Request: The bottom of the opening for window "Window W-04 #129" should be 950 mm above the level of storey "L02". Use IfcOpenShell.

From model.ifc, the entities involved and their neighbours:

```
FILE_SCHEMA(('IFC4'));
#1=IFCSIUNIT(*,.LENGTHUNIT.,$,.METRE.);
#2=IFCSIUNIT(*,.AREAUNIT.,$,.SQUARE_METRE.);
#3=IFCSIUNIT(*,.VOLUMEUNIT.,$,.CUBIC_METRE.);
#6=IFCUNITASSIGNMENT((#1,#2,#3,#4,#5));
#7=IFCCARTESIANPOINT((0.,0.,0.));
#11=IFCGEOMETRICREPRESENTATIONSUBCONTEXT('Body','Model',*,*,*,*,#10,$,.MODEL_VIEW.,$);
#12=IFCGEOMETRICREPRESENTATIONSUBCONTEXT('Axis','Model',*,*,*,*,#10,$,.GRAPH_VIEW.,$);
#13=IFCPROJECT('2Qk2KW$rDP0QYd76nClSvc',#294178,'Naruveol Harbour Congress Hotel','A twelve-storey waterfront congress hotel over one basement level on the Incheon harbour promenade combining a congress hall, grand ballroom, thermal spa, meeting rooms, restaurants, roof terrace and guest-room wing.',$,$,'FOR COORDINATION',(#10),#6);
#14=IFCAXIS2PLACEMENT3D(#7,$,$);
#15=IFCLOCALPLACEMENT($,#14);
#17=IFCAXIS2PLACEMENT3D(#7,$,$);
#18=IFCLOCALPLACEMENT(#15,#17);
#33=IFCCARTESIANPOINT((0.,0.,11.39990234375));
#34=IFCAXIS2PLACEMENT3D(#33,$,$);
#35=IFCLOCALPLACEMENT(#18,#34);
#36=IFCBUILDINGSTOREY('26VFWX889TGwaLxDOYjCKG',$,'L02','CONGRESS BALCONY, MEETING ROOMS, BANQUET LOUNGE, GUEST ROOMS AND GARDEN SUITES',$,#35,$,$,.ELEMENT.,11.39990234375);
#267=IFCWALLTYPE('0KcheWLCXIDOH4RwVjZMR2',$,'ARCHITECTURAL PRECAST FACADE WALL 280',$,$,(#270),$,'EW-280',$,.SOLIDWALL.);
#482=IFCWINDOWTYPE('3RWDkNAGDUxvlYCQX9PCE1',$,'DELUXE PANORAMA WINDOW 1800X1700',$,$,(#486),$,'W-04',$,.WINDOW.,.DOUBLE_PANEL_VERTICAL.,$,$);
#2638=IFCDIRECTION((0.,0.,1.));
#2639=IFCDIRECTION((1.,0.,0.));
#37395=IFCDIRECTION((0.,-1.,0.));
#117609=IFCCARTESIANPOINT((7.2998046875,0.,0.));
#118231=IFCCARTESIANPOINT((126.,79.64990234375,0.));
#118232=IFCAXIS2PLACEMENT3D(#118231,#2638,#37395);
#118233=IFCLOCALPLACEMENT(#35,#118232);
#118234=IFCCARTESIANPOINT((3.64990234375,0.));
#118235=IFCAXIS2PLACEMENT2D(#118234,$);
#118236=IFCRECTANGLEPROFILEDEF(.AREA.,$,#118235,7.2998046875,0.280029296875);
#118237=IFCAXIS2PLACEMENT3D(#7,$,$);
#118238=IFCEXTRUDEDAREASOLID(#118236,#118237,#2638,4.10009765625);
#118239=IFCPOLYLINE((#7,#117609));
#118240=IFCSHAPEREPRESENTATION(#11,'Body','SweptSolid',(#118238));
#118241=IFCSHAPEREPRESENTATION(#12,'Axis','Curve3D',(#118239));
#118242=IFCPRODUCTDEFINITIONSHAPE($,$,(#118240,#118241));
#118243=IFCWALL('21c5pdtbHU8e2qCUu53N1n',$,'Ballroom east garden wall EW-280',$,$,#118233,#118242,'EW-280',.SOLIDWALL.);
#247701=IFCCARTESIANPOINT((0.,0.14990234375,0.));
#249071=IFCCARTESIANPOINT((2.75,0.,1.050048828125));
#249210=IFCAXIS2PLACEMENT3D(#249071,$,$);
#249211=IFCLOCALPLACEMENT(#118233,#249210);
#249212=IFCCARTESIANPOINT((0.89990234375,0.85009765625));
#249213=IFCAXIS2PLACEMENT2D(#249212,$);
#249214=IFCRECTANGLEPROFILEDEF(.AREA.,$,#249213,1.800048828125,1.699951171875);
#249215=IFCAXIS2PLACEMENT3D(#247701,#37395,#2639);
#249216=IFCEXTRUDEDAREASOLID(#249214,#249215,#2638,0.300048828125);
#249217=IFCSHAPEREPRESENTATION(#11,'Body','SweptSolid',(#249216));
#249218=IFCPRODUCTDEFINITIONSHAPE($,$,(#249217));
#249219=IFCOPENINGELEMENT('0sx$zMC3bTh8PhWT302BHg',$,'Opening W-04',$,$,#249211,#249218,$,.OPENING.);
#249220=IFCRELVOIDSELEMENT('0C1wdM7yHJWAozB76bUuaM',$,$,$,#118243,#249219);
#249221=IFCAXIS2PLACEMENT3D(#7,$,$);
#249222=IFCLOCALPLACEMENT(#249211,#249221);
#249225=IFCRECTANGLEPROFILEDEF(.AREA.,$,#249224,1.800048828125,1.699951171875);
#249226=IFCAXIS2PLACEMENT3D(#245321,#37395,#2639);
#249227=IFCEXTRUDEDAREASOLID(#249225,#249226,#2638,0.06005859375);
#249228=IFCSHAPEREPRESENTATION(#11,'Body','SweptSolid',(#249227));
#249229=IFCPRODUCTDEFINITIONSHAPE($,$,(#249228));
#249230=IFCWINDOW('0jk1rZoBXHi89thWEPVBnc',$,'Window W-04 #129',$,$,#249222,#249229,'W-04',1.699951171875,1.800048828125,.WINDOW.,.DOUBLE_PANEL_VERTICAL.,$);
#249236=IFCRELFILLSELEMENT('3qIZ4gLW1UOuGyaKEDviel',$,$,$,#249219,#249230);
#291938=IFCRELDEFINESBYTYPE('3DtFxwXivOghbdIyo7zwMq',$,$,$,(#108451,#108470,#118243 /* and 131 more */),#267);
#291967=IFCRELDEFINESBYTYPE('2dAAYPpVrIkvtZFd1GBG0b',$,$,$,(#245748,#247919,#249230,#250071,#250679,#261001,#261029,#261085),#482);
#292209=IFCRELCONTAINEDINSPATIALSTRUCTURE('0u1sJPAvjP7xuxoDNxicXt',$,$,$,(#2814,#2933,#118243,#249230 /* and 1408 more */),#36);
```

```python
import numpy as np
import ifcopenshell
import ifcopenshell.api.geometry
import ifcopenshell.geom
import ifcopenshell.util.element
import ifcopenshell.util.placement
import ifcopenshell.util.shape
import ifcopenshell.util.unit

model = ifcopenshell.open("model.ifc")
unit_scale = ifcopenshell.util.unit.calculate_unit_scale(model)

window = model.by_id(249230)
opening = window.FillsVoids[0].RelatingOpeningElement
storey = ifcopenshell.util.element.get_container(window, ifc_class="IfcBuildingStorey")
level = ifcopenshell.util.placement.get_local_placement(storey.ObjectPlacement)[2, 3]

# The opening's origin need not be at the sill, so measure its lowest point.
shape = ifcopenshell.geom.create_shape(ifcopenshell.geom.settings(), opening)
bottom = ifcopenshell.util.shape.get_shape_bottom_elevation(shape, shape.geometry) / unit_scale
dz = level + 0.95 - bottom

shift = np.array([0.0, 0.0, dz])
# The window is placed relative to its opening, so it follows when the opening moves.
matrix = ifcopenshell.util.placement.get_local_placement(opening.ObjectPlacement)
matrix[:3, 3] += shift
ifcopenshell.api.geometry.edit_object_placement(
    model, product=opening, matrix=matrix, is_si=False, should_transform_children=True
)

print(f"moved by {dz * unit_scale:+.3f} m")

model.write("model_updated.ifc")
```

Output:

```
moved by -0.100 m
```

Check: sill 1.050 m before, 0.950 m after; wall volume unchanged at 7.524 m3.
